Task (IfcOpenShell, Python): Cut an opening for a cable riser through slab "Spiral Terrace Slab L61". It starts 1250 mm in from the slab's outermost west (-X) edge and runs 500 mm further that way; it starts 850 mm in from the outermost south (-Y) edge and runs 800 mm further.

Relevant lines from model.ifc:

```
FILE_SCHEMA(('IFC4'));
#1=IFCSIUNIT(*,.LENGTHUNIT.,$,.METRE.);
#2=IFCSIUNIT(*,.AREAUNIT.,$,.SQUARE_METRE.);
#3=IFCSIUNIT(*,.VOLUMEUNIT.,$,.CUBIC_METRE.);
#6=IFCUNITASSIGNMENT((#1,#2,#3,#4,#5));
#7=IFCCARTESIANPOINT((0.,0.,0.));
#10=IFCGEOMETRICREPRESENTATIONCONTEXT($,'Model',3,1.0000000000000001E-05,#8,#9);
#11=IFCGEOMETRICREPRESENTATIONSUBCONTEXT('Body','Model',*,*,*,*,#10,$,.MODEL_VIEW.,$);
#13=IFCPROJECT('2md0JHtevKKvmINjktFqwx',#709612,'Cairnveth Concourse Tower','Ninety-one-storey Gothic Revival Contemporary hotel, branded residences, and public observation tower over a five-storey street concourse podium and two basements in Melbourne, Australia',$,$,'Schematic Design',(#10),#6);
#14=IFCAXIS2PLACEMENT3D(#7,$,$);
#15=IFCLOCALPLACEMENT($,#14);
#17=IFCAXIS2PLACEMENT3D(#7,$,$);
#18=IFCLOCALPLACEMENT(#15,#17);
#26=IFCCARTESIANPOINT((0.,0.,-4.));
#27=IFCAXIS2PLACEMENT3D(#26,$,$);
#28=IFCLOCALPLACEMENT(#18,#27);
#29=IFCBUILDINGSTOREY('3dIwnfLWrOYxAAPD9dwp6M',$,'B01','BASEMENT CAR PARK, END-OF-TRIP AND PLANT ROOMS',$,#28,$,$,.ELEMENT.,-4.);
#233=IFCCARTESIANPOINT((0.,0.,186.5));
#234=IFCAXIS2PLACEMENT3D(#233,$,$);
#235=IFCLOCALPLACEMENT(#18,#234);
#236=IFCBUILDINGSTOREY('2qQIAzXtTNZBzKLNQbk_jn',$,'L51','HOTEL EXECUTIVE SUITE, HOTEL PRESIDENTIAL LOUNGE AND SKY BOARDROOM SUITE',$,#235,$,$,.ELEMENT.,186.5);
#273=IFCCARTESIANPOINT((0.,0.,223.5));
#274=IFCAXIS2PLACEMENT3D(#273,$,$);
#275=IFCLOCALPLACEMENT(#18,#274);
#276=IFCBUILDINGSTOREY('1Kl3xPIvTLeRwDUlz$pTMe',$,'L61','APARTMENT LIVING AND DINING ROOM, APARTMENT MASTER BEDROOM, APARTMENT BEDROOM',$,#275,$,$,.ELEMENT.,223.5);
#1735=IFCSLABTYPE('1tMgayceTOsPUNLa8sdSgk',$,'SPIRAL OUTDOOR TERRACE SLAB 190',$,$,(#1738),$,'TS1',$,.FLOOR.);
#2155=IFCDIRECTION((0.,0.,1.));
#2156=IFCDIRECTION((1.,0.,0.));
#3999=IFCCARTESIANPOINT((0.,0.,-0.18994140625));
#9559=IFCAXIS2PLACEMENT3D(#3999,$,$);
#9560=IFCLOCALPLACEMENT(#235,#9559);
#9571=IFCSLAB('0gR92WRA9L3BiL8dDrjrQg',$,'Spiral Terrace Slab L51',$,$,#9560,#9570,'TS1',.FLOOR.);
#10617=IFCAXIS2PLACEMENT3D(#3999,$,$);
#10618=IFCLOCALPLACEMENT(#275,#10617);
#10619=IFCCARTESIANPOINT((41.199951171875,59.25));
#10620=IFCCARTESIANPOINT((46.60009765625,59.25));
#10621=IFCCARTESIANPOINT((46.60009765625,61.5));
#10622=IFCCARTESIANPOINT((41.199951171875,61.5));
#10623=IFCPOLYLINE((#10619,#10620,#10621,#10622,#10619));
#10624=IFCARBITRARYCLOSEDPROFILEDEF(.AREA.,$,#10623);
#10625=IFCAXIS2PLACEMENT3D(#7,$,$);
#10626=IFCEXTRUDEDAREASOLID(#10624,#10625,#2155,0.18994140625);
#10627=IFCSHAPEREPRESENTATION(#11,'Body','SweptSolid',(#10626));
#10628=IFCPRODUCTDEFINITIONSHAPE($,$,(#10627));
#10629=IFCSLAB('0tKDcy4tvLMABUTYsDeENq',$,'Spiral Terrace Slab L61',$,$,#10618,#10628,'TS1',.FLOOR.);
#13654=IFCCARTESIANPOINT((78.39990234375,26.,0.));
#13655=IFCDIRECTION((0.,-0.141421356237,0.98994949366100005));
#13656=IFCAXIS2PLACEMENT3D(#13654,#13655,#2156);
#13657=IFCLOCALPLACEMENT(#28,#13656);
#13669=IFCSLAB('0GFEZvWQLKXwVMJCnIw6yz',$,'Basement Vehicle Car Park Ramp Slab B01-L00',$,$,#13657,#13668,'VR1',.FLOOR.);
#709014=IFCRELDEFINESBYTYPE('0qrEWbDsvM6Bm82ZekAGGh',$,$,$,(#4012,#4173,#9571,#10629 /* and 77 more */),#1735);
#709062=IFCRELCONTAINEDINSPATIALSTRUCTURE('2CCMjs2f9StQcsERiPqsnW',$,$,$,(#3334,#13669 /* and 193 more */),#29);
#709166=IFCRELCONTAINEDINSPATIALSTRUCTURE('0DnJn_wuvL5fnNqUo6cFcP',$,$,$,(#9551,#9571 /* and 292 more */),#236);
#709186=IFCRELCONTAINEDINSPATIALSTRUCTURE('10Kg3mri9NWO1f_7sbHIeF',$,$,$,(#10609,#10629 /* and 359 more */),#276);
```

```python
import numpy as np
import ifcopenshell
import ifcopenshell.api.feature
import ifcopenshell.api.geometry
import ifcopenshell.api.root
import ifcopenshell.geom
import ifcopenshell.util.placement
import ifcopenshell.util.representation
import ifcopenshell.util.shape
import ifcopenshell.util.unit

model = ifcopenshell.open("model.ifc")
unit_scale = ifcopenshell.util.unit.calculate_unit_scale(model)
settings = ifcopenshell.geom.settings()


def volume(element):
    """Net volume in cubic metres, openings subtracted."""
    shape = ifcopenshell.geom.create_shape(settings, element)
    return ifcopenshell.util.shape.get_volume(shape.geometry)


slab = model.by_guid("0tKDcy4tvLMABUTYsDeENq")
before = volume(slab)

# Extent in the slab's own axes, in metres. The edges named are its -X and -Y sides.
slab_shape = ifcopenshell.geom.create_shape(settings, slab)
vertices = ifcopenshell.util.shape.get_vertices(slab_shape.geometry)
x_min, y_min, bottom = vertices.min(axis=0)
top = vertices[:, 2].max()

opening = ifcopenshell.api.root.create_entity(model, ifc_class="IfcOpeningElement", name="Cable riser opening", predefined_type="OPENING")
context = ifcopenshell.util.representation.get_context(model, "Model", "Body", "MODEL_VIEW")
width, depth = 0.5, 0.8
outline = [(0.0, 0.0), (width, 0.0), (width, depth), (0.0, depth), (0.0, 0.0)]
# Overshoot both faces by 50 mm so the cut is clean.
shape = ifcopenshell.api.geometry.add_slab_representation(
    model, context=context, depth=top - bottom + 0.1, polyline=outline
)
ifcopenshell.api.geometry.assign_representation(model, product=opening, representation=shape)

matrix = ifcopenshell.util.placement.get_local_placement(slab.ObjectPlacement)
matrix[:, 3] = matrix @ np.append(np.array([x_min + 1.25, y_min + 0.85, bottom - 0.05]) / unit_scale, 1.0)
ifcopenshell.api.geometry.edit_object_placement(model, product=opening, matrix=matrix, is_si=False)
ifcopenshell.api.feature.add_feature(model, feature=opening, element=slab)

after = volume(slab)

print(f"slab volume {before:.3f} -> {after:.3f} m3")

model.write("model_v2.ifc")
```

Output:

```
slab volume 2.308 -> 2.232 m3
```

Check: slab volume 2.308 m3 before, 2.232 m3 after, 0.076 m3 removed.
